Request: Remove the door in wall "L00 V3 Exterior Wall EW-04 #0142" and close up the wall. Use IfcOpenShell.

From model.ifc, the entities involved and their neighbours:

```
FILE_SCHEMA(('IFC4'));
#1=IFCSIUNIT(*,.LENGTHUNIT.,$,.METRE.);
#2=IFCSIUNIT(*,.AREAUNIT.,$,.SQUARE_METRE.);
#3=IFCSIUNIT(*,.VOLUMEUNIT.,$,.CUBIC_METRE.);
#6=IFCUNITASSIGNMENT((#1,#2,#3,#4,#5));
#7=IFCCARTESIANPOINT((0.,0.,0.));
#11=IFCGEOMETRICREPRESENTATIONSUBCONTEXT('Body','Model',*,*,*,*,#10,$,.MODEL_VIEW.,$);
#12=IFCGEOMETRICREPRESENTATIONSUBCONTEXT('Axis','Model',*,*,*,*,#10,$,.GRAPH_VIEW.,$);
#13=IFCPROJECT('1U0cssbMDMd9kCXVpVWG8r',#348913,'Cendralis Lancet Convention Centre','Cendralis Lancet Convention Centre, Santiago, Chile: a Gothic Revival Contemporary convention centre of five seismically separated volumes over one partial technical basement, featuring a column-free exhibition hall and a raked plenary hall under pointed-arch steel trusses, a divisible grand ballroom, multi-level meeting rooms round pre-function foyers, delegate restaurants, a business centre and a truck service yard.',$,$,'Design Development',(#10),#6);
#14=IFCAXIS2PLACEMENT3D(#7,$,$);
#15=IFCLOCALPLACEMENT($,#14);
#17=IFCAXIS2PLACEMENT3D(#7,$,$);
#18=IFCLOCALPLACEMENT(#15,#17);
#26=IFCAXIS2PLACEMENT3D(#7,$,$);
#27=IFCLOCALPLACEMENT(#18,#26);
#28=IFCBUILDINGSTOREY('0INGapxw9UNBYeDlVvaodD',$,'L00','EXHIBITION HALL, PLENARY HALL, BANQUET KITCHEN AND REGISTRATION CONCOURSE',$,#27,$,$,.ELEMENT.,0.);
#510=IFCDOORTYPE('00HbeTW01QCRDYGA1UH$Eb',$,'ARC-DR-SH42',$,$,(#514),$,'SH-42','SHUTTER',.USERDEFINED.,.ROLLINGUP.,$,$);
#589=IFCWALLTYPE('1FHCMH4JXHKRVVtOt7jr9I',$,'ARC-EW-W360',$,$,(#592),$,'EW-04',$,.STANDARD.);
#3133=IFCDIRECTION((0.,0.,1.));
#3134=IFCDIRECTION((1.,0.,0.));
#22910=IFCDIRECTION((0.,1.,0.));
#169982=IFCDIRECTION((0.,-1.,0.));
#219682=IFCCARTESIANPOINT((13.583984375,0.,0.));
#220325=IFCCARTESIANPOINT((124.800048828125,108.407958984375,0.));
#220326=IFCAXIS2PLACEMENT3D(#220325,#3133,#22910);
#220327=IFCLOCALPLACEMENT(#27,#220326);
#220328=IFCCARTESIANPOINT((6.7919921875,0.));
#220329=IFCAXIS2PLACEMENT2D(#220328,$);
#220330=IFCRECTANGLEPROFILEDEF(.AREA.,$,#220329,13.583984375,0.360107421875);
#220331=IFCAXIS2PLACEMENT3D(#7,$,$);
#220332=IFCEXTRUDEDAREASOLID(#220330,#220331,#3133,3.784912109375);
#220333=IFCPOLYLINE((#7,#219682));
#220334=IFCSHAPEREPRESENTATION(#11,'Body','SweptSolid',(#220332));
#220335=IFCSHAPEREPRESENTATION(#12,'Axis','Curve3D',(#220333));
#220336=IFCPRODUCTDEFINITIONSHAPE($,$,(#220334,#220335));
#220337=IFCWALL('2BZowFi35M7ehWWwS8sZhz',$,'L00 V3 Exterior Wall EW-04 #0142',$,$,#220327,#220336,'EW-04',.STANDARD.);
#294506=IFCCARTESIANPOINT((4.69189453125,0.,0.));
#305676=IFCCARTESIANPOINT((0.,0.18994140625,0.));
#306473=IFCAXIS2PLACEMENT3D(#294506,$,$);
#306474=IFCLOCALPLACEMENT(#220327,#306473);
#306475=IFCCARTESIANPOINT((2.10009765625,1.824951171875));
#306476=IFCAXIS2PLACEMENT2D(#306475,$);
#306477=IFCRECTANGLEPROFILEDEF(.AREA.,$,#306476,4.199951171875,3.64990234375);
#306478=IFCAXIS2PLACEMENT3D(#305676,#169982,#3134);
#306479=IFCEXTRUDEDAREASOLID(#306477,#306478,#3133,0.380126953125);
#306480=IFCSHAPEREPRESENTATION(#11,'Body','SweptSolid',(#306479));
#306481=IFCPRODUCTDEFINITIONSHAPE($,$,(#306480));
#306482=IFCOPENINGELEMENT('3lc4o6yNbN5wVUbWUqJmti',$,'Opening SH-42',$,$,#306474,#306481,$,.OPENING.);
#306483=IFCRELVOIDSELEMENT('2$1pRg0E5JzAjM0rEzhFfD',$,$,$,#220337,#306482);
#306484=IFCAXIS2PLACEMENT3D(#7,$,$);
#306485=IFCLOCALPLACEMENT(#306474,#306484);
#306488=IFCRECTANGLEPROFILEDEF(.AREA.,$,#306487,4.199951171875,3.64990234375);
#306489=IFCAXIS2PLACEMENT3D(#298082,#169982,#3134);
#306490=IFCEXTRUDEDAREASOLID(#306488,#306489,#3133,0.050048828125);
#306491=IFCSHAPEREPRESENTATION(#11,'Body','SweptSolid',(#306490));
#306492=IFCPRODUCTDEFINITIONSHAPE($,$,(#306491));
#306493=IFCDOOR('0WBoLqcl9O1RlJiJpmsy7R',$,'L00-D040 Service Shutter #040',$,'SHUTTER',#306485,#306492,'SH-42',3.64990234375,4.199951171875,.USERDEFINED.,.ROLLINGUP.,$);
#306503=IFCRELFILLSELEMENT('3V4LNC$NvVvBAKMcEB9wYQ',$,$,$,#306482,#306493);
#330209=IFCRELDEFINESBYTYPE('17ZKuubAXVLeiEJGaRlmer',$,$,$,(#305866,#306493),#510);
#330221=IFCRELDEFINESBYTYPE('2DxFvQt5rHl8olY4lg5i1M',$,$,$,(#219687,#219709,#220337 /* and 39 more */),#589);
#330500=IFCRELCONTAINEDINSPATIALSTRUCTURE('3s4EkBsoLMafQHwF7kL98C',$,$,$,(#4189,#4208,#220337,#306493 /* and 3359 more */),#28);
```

```python
import ifcopenshell
import ifcopenshell.api.feature
import ifcopenshell.api.root
import ifcopenshell.geom
import ifcopenshell.util.shape

model = ifcopenshell.open("model.ifc")
settings = ifcopenshell.geom.settings()


def volume(element):
    """Net volume in cubic metres, openings subtracted."""
    shape = ifcopenshell.geom.create_shape(settings, element)
    return ifcopenshell.util.shape.get_volume(shape.geometry)


door = model.by_guid("0WBoLqcl9O1RlJiJpmsy7R")
opening = door.FillsVoids[0].RelatingOpeningElement
wall = opening.VoidsElements[0].RelatingBuildingElement
before = volume(wall)

ifcopenshell.api.root.remove_product(model, product=door)
ifcopenshell.api.feature.remove_feature(model, feature=opening)

after = volume(wall)

print(f"wall volume {before:.3f} -> {after:.3f} m3")

model.write("model-out.ifc")
```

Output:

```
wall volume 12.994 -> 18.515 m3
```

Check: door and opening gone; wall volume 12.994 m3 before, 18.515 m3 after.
